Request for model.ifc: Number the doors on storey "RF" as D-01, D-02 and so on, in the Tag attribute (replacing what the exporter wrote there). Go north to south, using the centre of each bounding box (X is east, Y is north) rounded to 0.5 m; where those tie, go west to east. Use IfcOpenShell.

First a look at what the model holds.

```python
import ifcopenshell
import ifcopenshell.util.element
import ifcopenshell.util.placement

model = ifcopenshell.open("model.ifc")
print(model.schema)
storey = next(s for s in model.by_type("IfcBuildingStorey") if s.Name == "RF")
doors = [e for e in ifcopenshell.util.element.get_decomposition(storey) if e.is_a("IfcDoor")]
for e in sorted(doors, key=lambda e: e.id()):
    origin = ifcopenshell.util.placement.get_local_placement(e.ObjectPlacement)[:3, 3]
    print(e.id(), e.Tag, e.Name, origin.round(2) + 0.0, sep=" | ")
```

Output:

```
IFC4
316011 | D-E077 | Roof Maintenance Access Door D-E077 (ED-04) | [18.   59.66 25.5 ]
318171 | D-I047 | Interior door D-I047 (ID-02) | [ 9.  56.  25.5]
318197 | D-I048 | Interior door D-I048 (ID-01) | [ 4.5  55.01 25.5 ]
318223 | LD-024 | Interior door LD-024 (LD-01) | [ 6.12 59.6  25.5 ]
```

```python
import ifcopenshell
import ifcopenshell.geom
import ifcopenshell.util.element
import ifcopenshell.util.shape

model = ifcopenshell.open("model.ifc")
settings = ifcopenshell.geom.settings()
settings.set("use-world-coords", True)


def centre(element):
    shape = ifcopenshell.geom.create_shape(settings, element)
    return ifcopenshell.util.shape.get_bbox_centroid(shape.geometry)


storey = next(s for s in model.by_type("IfcBuildingStorey") if s.Name == "RF")
doors = [e for e in ifcopenshell.util.element.get_decomposition(storey) if e.is_a("IfcDoor")]

# Insertion points can sit at a corner or the storey origin, so sort by the geometry (in metres).
centres = {e: centre(e) for e in doors}
doors.sort(key=lambda e: (-round(centres[e][1] / 0.5), centres[e][0]))

for i, e in enumerate(doors, start=1):
    number = f"D-{i:02d}"
    e.Tag = number
    print(e.id(), number)

model.write("model_edited.ifc")
```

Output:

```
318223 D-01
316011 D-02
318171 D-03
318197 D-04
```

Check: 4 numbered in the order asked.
